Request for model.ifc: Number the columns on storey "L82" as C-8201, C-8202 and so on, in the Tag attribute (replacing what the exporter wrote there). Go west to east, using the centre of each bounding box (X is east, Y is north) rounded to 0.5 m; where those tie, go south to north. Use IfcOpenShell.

First a look at what the model holds.

```python
import ifcopenshell
import ifcopenshell.util.element
import ifcopenshell.util.placement

model = ifcopenshell.open("model.ifc")
print(model.schema)
storey = next(s for s in model.by_type("IfcBuildingStorey") if s.Name == "L82")
columns = [e for e in ifcopenshell.util.element.get_decomposition(storey) if e.is_a("IfcColumn")]
for e in sorted(columns, key=lambda e: e.id()):
    origin = ifcopenshell.util.placement.get_local_placement(e.ObjectPlacement)[:3, 3]
    print(e.id(), e.Tag, e.Name, origin.round(2) + 0.0, sep=" | ")
```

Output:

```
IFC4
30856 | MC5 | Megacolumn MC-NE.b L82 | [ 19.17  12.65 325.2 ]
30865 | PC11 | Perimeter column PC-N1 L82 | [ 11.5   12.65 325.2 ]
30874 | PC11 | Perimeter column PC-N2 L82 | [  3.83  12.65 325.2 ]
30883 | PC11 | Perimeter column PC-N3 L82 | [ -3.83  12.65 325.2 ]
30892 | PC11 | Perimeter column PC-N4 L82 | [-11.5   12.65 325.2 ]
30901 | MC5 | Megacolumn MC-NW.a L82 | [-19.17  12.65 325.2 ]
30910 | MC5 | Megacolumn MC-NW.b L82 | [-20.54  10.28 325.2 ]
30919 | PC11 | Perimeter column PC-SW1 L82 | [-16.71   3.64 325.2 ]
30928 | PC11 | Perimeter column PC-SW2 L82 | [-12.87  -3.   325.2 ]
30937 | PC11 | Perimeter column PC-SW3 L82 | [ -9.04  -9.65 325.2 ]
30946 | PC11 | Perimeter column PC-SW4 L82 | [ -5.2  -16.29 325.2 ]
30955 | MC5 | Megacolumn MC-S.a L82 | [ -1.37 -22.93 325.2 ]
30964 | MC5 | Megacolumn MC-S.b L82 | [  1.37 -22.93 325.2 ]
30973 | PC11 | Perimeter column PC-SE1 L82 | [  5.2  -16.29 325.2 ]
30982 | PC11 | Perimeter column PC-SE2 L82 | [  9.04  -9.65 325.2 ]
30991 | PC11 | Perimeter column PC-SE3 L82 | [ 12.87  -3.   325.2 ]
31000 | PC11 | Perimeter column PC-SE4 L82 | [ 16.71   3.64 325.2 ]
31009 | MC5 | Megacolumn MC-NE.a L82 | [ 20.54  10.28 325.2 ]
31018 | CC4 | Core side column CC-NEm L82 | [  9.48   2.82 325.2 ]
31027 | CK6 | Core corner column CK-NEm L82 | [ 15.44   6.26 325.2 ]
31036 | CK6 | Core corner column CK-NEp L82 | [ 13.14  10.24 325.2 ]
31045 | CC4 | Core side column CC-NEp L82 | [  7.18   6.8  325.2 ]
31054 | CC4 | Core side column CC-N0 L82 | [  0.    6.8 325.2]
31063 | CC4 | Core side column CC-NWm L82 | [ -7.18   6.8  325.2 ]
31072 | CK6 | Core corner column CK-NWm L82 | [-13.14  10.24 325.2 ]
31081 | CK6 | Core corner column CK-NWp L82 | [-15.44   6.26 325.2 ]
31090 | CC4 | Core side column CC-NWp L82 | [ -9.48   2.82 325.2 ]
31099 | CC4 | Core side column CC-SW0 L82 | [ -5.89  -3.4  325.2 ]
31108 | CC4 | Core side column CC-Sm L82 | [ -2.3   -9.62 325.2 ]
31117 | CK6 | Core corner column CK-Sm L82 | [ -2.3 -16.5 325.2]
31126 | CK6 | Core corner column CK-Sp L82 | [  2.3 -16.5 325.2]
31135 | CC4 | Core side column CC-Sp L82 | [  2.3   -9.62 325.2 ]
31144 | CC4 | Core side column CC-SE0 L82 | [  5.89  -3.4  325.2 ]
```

```python
import ifcopenshell
import ifcopenshell.geom
import ifcopenshell.util.element
import ifcopenshell.util.shape

model = ifcopenshell.open("model.ifc")
settings = ifcopenshell.geom.settings()
settings.set("use-world-coords", True)


def centre(element):
    shape = ifcopenshell.geom.create_shape(settings, element)
    return ifcopenshell.util.shape.get_bbox_centroid(shape.geometry)


storey = next(s for s in model.by_type("IfcBuildingStorey") if s.Name == "L82")
columns = [e for e in ifcopenshell.util.element.get_decomposition(storey) if e.is_a("IfcColumn")]

# Insertion points can sit at a corner or the storey origin, so sort by the geometry (in metres).
centres = {e: centre(e) for e in columns}
columns.sort(key=lambda e: (round(centres[e][0] / 0.5), centres[e][1]))

for i, e in enumerate(columns, start=1):
    number = f"C-82{i:02d}"
    e.Tag = number
    print(e.id(), number)

model.write("model-out.ifc")
```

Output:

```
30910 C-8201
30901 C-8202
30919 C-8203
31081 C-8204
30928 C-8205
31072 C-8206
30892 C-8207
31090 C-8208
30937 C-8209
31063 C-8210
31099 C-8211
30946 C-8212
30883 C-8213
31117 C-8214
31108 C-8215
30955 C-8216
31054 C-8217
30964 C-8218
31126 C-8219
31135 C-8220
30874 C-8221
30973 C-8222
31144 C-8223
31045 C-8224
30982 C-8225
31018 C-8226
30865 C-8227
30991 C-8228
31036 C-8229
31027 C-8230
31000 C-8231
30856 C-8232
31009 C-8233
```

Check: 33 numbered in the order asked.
